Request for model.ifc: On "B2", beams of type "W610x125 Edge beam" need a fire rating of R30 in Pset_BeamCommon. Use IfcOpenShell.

First a look at what the model holds.

```python
import ifcopenshell
import ifcopenshell.util.element

model = ifcopenshell.open("model.ifc")
print(model.schema)
storey = next(s for s in model.by_type("IfcBuildingStorey") if s.Name == "B2")
beams = [e for e in ifcopenshell.util.element.get_decomposition(storey) if e.is_a("IfcBeam")]
seen = {}
for e in beams:
    element_type = ifcopenshell.util.element.get_type(e)
    key = (element_type.Name if element_type != e and element_type else None, ifcopenshell.util.element.get_pset(e, "Pset_BeamCommon", "FireRating"))
    seen[key] = seen.get(key, 0) + 1
for (name, value), count in sorted(seen.items(), key=str):
    print(count, "x", name, "|", value)
```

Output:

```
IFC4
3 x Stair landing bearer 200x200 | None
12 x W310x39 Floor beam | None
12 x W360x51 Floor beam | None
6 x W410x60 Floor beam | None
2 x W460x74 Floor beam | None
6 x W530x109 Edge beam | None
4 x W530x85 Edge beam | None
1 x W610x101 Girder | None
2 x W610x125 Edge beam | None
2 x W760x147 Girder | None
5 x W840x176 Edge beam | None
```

```python
import ifcopenshell
import ifcopenshell.api.pset
import ifcopenshell.util.element

model = ifcopenshell.open("model.ifc")

storey = next(s for s in model.by_type("IfcBuildingStorey") if s.Name == "B2")
beams = [e for e in ifcopenshell.util.element.get_decomposition(storey) if e.is_a("IfcBeam")]

count = 0
for e in beams:
    element_type = ifcopenshell.util.element.get_type(e)
    if element_type in (None, e) or element_type.Name != "W610x125 Edge beam":
        continue
    found = ifcopenshell.util.element.get_pset(e, "Pset_BeamCommon", should_inherit=False)
    if found:
        pset = model.by_id(found["id"])
        if len(ifcopenshell.util.element.get_elements_by_pset(pset)) > 1:
            pset = ifcopenshell.api.pset.unshare_pset(model, products=[e], pset=pset)[0]
    else:
        pset = ifcopenshell.api.pset.add_pset(model, product=e, name="Pset_BeamCommon")
    ifcopenshell.api.pset.edit_pset(model, pset=pset, properties={"FireRating": "R30"})
    count += 1

print(count, "beams updated")

model.write("model_updated.ifc")
```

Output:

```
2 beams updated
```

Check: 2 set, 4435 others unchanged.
